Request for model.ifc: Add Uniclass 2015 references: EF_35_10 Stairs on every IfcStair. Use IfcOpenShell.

First a look at what the model holds.

```python
import ifcopenshell

model = ifcopenshell.open("model.ifc")
print(model.schema)
print("classifications:", [c.Name for c in model.by_type("IfcClassification")])
for ifc_class in ("IfcDoor", "IfcRoof", "IfcStair", "IfcWall", "IfcWindow"):
    print(ifc_class, len(model.by_type(ifc_class)))
```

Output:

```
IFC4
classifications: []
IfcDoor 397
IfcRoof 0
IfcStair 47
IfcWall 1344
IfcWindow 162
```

```python
import ifcopenshell
import ifcopenshell.api.classification

model = ifcopenshell.open("model.ifc")

system = ifcopenshell.api.classification.add_classification(model, classification="Uniclass 2015")

codes = {
    "IfcStair": ("EF_35_10", "Stairs"),
}
for ifc_class, (code, name) in codes.items():
    products = model.by_type(ifc_class)
    ifcopenshell.api.classification.add_reference(
        model, products=products, classification=system, identification=code, name=name
    )
    print(code, len(products))

model.write("model_rev.ifc")
```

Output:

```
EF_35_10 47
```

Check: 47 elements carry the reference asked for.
